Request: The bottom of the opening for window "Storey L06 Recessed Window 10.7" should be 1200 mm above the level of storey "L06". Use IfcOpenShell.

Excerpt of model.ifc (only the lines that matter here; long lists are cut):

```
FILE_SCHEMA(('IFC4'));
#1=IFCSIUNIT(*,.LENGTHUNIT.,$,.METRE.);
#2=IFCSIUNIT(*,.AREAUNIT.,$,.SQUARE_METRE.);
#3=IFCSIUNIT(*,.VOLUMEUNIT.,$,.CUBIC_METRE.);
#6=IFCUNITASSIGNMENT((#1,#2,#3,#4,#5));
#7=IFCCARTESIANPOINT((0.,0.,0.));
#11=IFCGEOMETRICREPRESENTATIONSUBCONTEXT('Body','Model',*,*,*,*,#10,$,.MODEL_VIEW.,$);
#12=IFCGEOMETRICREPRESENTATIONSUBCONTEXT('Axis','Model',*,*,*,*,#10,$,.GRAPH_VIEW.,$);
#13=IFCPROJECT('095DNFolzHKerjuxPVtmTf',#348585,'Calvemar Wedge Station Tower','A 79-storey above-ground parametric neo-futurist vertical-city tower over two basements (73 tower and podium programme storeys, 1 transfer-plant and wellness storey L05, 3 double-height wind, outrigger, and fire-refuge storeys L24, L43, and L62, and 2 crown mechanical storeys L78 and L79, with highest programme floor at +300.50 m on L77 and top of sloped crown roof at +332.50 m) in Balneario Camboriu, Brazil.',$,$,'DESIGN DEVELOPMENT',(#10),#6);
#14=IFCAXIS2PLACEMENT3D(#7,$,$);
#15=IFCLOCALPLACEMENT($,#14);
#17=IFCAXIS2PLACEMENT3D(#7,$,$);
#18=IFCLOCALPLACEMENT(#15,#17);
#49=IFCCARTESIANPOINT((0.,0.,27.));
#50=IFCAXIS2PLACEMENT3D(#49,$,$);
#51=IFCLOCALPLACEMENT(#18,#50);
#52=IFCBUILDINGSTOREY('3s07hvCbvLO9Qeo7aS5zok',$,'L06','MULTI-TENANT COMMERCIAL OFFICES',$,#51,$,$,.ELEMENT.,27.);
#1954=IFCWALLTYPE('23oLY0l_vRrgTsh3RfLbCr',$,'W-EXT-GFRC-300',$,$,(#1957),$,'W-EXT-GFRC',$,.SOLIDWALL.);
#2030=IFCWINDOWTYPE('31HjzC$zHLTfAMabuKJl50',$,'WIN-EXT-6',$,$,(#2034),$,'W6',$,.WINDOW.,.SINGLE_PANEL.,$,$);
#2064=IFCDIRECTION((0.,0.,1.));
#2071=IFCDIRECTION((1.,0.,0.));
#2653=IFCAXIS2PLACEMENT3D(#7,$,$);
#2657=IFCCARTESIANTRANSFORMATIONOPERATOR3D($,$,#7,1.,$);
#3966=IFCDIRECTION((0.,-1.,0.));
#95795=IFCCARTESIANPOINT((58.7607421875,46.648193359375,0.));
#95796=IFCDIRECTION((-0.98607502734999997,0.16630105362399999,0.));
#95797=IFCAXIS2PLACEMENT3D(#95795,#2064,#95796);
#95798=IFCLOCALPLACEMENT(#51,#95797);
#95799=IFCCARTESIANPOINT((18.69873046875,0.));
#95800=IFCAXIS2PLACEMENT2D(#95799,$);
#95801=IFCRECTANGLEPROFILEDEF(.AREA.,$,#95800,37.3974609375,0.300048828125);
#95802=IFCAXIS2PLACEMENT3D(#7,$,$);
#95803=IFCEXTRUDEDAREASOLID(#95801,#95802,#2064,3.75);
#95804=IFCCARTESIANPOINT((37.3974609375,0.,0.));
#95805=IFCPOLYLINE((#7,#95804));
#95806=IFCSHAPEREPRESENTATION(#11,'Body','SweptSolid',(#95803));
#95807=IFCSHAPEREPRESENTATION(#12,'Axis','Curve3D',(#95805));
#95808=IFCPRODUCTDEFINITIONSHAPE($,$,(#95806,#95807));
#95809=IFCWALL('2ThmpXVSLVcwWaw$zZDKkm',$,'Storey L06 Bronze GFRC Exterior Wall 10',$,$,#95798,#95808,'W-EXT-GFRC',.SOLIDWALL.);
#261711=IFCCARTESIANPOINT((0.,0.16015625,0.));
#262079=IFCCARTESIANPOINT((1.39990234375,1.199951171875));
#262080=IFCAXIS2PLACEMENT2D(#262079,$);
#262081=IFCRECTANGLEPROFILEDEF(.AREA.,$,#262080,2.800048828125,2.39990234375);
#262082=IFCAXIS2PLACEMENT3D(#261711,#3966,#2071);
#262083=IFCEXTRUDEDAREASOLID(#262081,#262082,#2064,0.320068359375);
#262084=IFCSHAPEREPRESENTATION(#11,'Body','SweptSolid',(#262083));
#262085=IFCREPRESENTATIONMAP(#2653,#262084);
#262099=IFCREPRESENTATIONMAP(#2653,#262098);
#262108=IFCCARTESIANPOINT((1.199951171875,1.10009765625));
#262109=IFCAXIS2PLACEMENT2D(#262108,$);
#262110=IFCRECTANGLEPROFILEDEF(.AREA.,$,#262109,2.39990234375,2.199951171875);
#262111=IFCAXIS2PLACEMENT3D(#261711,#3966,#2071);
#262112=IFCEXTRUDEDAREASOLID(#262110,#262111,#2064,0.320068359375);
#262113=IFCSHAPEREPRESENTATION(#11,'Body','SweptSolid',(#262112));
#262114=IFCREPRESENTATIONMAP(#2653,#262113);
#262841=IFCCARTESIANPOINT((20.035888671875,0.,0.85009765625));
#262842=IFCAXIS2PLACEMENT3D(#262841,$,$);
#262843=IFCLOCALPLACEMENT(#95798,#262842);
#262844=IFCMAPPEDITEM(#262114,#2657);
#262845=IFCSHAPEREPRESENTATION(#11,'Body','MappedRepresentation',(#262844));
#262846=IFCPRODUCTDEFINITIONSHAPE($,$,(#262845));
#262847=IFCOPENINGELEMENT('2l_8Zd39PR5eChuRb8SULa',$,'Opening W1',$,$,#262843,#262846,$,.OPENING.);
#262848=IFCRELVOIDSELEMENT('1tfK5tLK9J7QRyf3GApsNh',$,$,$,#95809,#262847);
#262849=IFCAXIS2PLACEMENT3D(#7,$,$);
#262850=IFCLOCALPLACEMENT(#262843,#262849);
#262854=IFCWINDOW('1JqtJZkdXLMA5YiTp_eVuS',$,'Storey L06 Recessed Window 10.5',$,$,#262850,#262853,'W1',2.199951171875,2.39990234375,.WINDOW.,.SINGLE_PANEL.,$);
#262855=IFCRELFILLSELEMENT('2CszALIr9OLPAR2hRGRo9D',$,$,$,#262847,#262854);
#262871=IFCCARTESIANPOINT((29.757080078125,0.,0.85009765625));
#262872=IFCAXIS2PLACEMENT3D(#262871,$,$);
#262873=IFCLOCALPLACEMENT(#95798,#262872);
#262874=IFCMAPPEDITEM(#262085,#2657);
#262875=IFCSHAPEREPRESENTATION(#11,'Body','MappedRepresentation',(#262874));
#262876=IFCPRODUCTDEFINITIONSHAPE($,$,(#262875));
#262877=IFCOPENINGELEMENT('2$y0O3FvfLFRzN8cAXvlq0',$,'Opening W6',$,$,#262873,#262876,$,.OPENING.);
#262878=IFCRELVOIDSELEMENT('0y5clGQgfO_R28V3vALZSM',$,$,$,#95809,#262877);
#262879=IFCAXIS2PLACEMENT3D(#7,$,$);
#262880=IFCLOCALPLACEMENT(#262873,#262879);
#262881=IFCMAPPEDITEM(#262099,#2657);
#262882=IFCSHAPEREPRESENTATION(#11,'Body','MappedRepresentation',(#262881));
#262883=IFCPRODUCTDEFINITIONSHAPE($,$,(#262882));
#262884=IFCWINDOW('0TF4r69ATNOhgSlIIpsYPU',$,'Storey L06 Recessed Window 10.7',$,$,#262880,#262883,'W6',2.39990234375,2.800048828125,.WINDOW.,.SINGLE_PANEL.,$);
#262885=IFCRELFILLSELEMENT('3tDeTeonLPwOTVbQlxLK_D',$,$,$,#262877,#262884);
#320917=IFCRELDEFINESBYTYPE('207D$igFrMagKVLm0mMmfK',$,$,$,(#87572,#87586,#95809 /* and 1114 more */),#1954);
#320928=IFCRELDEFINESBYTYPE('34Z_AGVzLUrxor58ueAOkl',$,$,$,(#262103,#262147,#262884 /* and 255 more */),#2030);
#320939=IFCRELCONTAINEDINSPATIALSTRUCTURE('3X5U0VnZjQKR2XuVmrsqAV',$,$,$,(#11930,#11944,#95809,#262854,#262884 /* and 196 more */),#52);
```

```python
import numpy as np
import ifcopenshell
import ifcopenshell.api.geometry
import ifcopenshell.geom
import ifcopenshell.util.element
import ifcopenshell.util.placement
import ifcopenshell.util.shape
import ifcopenshell.util.unit

model = ifcopenshell.open("model.ifc")
unit_scale = ifcopenshell.util.unit.calculate_unit_scale(model)

window = model.by_guid("0TF4r69ATNOhgSlIIpsYPU")
opening = window.FillsVoids[0].RelatingOpeningElement
storey = ifcopenshell.util.element.get_container(window, ifc_class="IfcBuildingStorey")
level = ifcopenshell.util.placement.get_local_placement(storey.ObjectPlacement)[2, 3]

# The opening's origin need not be at the sill, so measure its lowest point.
shape = ifcopenshell.geom.create_shape(ifcopenshell.geom.settings(), opening)
bottom = ifcopenshell.util.shape.get_shape_bottom_elevation(shape, shape.geometry) / unit_scale
dz = level + 1.2 / unit_scale - bottom

shift = np.array([0.0, 0.0, dz])
# The window is placed relative to its opening, so it follows when the opening moves.
matrix = ifcopenshell.util.placement.get_local_placement(opening.ObjectPlacement)
matrix[:3, 3] += shift
ifcopenshell.api.geometry.edit_object_placement(
    model, product=opening, matrix=matrix, is_si=False, should_transform_children=True
)

print(f"moved by {dz * unit_scale:+.3f} m")

model.write("model_updated.ifc")
```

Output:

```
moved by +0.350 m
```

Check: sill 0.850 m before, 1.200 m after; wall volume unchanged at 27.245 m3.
